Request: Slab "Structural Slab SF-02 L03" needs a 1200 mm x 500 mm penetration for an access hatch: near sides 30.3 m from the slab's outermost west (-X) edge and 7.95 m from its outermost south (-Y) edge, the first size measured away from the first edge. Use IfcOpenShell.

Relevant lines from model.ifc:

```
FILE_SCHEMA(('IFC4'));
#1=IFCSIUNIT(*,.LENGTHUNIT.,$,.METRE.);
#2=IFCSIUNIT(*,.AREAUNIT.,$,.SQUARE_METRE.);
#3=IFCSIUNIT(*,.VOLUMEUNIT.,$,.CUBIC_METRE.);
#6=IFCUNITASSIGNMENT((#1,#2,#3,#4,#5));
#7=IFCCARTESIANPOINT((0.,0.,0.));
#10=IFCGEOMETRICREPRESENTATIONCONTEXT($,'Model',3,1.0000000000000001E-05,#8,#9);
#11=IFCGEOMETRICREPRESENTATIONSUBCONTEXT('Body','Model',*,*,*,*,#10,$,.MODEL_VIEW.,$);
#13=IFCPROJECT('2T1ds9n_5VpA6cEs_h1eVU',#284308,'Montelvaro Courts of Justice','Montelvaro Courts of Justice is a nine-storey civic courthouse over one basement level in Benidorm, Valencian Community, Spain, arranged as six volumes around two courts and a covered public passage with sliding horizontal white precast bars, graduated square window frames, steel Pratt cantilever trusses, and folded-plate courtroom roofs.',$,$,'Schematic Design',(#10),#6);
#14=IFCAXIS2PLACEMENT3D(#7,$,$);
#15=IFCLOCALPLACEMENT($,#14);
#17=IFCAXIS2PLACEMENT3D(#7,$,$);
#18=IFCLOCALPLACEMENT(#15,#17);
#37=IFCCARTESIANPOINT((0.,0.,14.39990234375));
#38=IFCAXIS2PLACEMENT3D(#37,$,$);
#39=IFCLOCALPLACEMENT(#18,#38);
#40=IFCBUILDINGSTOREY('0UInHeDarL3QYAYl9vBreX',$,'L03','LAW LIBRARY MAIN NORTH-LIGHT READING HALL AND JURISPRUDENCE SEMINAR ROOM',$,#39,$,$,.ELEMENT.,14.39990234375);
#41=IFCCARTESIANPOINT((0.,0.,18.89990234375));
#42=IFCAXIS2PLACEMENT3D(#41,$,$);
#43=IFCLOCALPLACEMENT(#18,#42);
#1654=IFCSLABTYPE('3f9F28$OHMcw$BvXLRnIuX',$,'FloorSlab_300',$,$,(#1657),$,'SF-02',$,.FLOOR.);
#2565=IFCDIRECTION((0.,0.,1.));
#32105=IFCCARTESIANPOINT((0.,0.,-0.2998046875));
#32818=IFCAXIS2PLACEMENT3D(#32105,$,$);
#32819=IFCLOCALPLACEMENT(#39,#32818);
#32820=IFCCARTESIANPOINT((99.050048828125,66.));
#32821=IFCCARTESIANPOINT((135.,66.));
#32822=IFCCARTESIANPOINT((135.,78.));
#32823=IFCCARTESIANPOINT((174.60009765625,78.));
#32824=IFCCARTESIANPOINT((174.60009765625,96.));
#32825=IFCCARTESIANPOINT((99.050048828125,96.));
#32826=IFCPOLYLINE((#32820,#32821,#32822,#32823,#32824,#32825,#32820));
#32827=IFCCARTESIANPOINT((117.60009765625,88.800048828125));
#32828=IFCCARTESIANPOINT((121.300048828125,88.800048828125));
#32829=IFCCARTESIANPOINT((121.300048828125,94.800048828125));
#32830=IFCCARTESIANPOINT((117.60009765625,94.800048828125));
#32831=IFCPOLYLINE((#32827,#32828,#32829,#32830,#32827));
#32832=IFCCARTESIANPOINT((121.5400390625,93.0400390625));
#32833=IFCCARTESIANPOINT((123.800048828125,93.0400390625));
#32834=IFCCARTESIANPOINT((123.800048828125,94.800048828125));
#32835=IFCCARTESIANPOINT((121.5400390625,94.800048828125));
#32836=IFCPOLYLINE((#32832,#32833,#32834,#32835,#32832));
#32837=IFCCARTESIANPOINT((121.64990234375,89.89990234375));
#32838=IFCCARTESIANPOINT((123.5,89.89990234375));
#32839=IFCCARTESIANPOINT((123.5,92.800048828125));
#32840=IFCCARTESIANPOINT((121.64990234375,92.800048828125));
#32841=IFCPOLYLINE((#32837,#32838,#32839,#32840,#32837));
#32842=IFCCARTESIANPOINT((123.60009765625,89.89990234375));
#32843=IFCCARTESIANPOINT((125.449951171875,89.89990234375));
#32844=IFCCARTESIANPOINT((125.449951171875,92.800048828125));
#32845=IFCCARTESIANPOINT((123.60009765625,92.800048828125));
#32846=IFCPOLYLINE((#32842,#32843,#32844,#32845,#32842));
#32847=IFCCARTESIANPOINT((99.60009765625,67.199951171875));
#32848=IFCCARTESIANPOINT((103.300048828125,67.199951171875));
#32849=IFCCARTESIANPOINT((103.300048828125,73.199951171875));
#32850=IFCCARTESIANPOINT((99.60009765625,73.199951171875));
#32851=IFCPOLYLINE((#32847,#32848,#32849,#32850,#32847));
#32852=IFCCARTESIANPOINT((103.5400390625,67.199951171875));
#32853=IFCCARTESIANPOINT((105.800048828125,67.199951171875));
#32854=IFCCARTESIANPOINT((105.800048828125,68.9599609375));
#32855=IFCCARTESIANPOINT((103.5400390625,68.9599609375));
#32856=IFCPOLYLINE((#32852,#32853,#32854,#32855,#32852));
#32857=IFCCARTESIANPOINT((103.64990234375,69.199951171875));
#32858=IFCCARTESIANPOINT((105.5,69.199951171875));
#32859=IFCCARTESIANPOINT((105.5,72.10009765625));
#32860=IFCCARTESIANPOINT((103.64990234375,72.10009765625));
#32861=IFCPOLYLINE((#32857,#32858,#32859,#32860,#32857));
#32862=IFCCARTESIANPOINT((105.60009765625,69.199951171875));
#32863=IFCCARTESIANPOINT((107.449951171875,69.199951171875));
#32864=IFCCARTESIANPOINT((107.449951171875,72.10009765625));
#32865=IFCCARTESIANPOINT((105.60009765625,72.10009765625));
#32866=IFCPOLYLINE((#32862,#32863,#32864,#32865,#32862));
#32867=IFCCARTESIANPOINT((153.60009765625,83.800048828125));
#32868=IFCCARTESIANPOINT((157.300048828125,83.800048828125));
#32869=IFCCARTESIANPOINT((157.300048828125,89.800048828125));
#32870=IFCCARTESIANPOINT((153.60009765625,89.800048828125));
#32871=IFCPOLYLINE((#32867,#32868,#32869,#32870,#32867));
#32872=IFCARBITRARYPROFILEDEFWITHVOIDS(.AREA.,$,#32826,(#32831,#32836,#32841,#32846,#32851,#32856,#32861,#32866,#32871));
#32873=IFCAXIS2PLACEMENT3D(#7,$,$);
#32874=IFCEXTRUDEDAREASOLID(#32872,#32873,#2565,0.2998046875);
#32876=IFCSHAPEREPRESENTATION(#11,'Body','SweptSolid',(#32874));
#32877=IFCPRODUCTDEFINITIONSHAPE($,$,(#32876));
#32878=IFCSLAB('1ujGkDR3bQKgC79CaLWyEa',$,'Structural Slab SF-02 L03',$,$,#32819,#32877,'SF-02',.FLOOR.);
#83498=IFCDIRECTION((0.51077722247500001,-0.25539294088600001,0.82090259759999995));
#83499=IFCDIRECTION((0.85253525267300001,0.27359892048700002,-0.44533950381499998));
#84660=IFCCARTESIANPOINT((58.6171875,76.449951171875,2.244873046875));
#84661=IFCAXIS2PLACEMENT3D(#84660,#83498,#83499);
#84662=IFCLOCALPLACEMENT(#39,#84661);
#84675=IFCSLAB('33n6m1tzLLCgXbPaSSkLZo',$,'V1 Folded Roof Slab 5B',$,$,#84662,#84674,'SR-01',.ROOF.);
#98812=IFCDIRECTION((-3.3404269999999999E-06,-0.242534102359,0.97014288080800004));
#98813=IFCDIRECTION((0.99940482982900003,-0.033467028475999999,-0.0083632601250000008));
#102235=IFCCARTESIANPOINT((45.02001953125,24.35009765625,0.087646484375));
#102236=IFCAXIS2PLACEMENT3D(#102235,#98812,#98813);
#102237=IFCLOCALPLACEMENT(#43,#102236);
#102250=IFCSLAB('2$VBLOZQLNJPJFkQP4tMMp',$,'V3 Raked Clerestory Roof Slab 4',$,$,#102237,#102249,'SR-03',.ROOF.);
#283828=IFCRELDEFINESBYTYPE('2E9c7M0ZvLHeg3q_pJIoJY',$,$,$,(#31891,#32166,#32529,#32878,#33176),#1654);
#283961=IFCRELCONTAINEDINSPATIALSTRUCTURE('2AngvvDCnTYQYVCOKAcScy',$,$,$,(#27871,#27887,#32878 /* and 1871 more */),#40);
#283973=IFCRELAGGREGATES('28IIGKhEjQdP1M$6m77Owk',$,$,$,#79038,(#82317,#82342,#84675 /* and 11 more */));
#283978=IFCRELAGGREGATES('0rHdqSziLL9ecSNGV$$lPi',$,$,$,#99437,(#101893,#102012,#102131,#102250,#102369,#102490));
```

```python
import numpy as np
import ifcopenshell
import ifcopenshell.api.feature
import ifcopenshell.api.geometry
import ifcopenshell.api.root
import ifcopenshell.geom
import ifcopenshell.util.placement
import ifcopenshell.util.representation
import ifcopenshell.util.shape
import ifcopenshell.util.unit

model = ifcopenshell.open("model.ifc")
unit_scale = ifcopenshell.util.unit.calculate_unit_scale(model)
settings = ifcopenshell.geom.settings()


def volume(element):
    """Net volume in cubic metres, openings subtracted."""
    shape = ifcopenshell.geom.create_shape(settings, element)
    return ifcopenshell.util.shape.get_volume(shape.geometry)


slab = model.by_id(32878)
before = volume(slab)

# Extent in the slab's own axes, in metres. The edges named are its -X and -Y sides.
slab_shape = ifcopenshell.geom.create_shape(settings, slab)
vertices = ifcopenshell.util.shape.get_vertices(slab_shape.geometry)
x_min, y_min, bottom = vertices.min(axis=0)
top = vertices[:, 2].max()

opening = ifcopenshell.api.root.create_entity(model, ifc_class="IfcOpeningElement", name="Access hatch opening", predefined_type="OPENING")
context = ifcopenshell.util.representation.get_context(model, "Model", "Body", "MODEL_VIEW")
width, depth = 1.2, 0.5
outline = [(0.0, 0.0), (width, 0.0), (width, depth), (0.0, depth), (0.0, 0.0)]
# Overshoot both faces by 50 mm so the cut is clean.
shape = ifcopenshell.api.geometry.add_slab_representation(
    model, context=context, depth=top - bottom + 0.1, polyline=outline
)
ifcopenshell.api.geometry.assign_representation(model, product=opening, representation=shape)

matrix = ifcopenshell.util.placement.get_local_placement(slab.ObjectPlacement)
matrix[:, 3] = matrix @ np.append(np.array([x_min + 30.3, y_min + 7.95, bottom - 0.05]) / unit_scale, 1.0)
ifcopenshell.api.geometry.edit_object_placement(model, product=opening, matrix=matrix, is_si=False)
ifcopenshell.api.feature.add_feature(model, feature=opening, element=slab)

after = volume(slab)

print(f"slab volume {before:.3f} -> {after:.3f} m3")

model.write("model_rev.ifc")
```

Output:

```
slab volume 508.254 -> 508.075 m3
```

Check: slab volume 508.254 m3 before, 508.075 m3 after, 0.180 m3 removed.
